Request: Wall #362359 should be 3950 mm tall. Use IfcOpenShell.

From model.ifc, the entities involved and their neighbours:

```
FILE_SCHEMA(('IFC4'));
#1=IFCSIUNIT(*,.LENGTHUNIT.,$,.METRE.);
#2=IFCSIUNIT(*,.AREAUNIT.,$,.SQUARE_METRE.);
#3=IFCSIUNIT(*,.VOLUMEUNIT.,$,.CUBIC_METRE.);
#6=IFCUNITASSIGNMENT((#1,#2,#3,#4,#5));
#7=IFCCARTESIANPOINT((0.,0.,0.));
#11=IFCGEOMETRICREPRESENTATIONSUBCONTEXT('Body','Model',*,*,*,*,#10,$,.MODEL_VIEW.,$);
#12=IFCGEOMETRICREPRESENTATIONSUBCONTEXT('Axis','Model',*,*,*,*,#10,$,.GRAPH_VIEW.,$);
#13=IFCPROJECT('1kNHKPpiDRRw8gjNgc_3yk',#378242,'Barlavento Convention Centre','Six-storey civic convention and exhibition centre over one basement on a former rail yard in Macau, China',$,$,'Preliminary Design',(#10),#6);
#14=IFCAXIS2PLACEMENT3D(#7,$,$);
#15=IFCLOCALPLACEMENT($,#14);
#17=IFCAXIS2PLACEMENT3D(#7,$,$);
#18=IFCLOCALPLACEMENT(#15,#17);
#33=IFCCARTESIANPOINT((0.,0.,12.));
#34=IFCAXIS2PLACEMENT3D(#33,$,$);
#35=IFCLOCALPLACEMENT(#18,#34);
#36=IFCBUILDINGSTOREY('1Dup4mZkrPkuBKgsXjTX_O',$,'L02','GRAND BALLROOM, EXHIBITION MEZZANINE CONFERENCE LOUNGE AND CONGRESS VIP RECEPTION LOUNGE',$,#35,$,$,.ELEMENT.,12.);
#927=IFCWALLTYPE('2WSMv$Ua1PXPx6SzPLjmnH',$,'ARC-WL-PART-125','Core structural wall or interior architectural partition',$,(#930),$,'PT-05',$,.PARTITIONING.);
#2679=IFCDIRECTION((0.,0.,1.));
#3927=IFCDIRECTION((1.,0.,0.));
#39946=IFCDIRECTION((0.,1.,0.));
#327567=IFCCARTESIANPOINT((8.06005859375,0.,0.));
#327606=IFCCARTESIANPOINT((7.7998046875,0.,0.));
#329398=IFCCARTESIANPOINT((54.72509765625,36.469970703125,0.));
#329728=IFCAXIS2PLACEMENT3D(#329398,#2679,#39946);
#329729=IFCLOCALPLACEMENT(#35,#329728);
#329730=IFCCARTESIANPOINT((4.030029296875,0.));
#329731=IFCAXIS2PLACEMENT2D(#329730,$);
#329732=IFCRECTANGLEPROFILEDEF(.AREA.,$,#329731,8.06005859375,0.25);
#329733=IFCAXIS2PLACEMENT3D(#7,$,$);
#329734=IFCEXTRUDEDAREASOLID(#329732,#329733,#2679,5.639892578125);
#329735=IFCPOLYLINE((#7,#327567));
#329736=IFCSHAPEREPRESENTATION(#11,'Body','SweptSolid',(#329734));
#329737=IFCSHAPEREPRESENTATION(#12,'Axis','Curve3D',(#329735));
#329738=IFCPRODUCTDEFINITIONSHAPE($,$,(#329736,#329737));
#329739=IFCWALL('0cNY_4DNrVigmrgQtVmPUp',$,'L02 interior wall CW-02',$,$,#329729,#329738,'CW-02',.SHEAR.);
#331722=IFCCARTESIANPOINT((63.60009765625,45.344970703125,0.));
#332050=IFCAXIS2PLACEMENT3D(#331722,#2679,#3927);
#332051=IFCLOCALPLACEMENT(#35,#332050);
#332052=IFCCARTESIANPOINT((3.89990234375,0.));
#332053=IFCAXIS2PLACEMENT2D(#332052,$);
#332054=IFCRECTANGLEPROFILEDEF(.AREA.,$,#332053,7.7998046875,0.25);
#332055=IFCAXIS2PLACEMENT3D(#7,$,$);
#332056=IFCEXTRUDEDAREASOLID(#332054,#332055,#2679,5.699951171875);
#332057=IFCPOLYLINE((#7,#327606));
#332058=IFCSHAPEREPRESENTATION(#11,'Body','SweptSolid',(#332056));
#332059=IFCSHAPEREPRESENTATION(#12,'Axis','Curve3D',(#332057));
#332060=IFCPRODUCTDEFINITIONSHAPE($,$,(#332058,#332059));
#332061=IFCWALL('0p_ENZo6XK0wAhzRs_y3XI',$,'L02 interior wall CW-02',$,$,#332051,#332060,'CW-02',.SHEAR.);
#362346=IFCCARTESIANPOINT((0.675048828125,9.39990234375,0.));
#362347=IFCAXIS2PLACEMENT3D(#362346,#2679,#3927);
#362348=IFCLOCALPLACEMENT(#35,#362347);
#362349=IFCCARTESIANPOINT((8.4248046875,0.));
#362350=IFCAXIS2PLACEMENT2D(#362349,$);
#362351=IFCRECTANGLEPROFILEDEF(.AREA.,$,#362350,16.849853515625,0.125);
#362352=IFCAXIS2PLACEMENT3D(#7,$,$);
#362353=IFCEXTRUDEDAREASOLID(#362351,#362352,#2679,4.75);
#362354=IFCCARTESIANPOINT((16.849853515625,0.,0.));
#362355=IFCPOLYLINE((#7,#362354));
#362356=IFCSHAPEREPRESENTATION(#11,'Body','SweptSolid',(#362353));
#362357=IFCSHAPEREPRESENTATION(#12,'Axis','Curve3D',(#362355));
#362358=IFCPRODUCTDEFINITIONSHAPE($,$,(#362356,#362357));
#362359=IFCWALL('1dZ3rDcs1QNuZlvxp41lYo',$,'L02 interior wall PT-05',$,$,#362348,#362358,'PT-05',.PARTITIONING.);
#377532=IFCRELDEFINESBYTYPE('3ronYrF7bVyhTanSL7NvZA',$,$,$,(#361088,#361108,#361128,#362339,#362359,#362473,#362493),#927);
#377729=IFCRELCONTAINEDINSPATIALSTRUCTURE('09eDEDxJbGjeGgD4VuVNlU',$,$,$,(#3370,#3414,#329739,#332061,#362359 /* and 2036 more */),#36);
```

```python
import ifcopenshell
import ifcopenshell.geom
import ifcopenshell.util.representation
import ifcopenshell.util.shape
import ifcopenshell.util.unit

model = ifcopenshell.open("model.ifc")
unit_scale = ifcopenshell.util.unit.calculate_unit_scale(model)
settings = ifcopenshell.geom.settings()


def volume(element):
    """Net volume in cubic metres, openings subtracted."""
    shape = ifcopenshell.geom.create_shape(settings, element)
    return ifcopenshell.util.shape.get_volume(shape.geometry)


wall = model.by_guid("1dZ3rDcs1QNuZlvxp41lYo")
before = volume(wall)

body = ifcopenshell.util.representation.get_representation(wall, "Model", "Body")
solid = body.Items[0]
old_height = solid.Depth
solid.Depth = 3.95 / unit_scale
after = volume(wall)

print(f"height {old_height:g} -> {solid.Depth:g}, volume {before:.3f} -> {after:.3f} m3")

model.write("model-out.ifc")
```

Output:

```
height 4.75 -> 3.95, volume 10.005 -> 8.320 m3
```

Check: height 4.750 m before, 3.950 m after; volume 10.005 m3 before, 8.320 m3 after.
